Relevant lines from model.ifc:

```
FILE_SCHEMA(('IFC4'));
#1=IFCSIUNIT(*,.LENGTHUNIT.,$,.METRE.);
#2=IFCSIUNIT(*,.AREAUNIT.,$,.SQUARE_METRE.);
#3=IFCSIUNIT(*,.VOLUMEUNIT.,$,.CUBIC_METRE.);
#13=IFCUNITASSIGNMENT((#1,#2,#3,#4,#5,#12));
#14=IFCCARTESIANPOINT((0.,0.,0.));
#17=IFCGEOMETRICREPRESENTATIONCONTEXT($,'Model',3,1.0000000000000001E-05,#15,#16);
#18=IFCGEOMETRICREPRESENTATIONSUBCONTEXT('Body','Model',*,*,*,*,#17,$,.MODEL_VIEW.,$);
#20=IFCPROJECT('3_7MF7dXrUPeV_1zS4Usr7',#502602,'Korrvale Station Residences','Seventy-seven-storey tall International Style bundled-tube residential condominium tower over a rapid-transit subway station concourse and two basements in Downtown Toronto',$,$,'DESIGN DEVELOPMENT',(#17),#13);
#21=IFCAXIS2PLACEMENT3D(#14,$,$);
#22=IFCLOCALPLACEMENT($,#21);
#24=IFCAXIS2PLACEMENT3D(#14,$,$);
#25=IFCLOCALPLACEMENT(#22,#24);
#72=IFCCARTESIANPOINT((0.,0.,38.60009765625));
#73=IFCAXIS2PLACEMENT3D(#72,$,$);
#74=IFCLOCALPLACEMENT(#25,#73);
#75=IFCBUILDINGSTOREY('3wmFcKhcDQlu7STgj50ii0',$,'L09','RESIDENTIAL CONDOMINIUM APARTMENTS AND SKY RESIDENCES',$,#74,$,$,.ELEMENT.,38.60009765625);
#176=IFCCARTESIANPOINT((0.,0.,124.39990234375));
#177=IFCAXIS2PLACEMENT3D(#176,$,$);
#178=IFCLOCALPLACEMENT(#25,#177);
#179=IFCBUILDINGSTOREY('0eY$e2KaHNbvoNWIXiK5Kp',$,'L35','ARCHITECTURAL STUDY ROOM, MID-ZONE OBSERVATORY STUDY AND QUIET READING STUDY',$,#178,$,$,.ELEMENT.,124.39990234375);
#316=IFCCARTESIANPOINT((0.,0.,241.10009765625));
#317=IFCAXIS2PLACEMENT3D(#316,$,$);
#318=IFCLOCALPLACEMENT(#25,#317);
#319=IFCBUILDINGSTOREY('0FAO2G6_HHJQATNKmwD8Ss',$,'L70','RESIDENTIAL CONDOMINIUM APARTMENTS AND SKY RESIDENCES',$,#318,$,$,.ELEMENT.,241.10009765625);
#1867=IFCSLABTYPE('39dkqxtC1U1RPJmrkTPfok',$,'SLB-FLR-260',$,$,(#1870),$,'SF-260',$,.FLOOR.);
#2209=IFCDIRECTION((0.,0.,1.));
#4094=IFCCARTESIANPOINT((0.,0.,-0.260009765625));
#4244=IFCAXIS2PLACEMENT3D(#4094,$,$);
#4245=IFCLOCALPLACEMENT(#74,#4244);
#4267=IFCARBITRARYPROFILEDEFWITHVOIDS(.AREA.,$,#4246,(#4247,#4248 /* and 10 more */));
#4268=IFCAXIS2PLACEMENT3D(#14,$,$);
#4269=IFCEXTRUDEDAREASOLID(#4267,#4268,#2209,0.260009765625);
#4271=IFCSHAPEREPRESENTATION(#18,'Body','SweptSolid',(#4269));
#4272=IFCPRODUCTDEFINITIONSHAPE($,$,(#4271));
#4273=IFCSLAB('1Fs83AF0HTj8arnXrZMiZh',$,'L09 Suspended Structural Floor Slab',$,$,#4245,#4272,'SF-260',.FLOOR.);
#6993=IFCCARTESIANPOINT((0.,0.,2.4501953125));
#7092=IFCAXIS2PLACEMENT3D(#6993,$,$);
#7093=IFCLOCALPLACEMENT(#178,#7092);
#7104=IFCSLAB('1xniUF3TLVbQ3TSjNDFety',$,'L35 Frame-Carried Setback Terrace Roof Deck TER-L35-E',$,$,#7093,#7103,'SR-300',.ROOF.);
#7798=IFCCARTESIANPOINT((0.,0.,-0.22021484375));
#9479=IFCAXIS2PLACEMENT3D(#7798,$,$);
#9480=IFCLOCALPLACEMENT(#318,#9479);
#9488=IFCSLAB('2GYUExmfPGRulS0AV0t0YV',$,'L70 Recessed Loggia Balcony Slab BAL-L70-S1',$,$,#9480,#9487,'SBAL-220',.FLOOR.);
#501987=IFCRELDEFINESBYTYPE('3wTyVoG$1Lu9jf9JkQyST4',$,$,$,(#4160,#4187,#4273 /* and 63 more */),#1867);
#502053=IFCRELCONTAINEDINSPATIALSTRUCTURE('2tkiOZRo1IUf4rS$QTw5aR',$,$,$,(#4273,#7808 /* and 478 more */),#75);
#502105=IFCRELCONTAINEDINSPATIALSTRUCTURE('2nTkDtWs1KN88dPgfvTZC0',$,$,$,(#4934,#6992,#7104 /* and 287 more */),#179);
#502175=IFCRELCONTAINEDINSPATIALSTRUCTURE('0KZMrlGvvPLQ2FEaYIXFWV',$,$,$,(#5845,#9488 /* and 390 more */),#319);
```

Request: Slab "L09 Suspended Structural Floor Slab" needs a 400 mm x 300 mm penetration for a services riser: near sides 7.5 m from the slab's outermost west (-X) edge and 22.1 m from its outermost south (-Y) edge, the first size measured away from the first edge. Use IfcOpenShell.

```python
import numpy as np
import ifcopenshell
import ifcopenshell.api.feature
import ifcopenshell.api.geometry
import ifcopenshell.api.root
import ifcopenshell.geom
import ifcopenshell.util.placement
import ifcopenshell.util.representation
import ifcopenshell.util.shape
import ifcopenshell.util.unit

model = ifcopenshell.open("model.ifc")
unit_scale = ifcopenshell.util.unit.calculate_unit_scale(model)
settings = ifcopenshell.geom.settings()


def volume(element):
    """Net volume in cubic metres, openings subtracted."""
    shape = ifcopenshell.geom.create_shape(settings, element)
    return ifcopenshell.util.shape.get_volume(shape.geometry)


slab = model.by_id(4273)
before = volume(slab)

# Extent in the slab's own axes, in metres. The edges named are its -X and -Y sides.
slab_shape = ifcopenshell.geom.create_shape(settings, slab)
vertices = ifcopenshell.util.shape.get_vertices(slab_shape.geometry)
x_min, y_min, bottom = vertices.min(axis=0)
top = vertices[:, 2].max()

opening = ifcopenshell.api.root.create_entity(model, ifc_class="IfcOpeningElement", name="Services riser opening", predefined_type="OPENING")
context = ifcopenshell.util.representation.get_context(model, "Model", "Body", "MODEL_VIEW")
width, depth = 0.4, 0.3
outline = [(0.0, 0.0), (width, 0.0), (width, depth), (0.0, depth), (0.0, 0.0)]
# Overshoot both faces by 50 mm so the cut is clean.
shape = ifcopenshell.api.geometry.add_slab_representation(
    model, context=context, depth=top - bottom + 0.1, polyline=outline
)
ifcopenshell.api.geometry.assign_representation(model, product=opening, representation=shape)

matrix = ifcopenshell.util.placement.get_local_placement(slab.ObjectPlacement)
matrix[:, 3] = matrix @ np.append(np.array([x_min + 7.5, y_min + 22.1, bottom - 0.05]) / unit_scale, 1.0)
ifcopenshell.api.geometry.edit_object_placement(model, product=opening, matrix=matrix, is_si=False)
ifcopenshell.api.feature.add_feature(model, feature=opening, element=slab)

after = volume(slab)

print(f"slab volume {before:.3f} -> {after:.3f} m3")

model.write("model-out.ifc")
```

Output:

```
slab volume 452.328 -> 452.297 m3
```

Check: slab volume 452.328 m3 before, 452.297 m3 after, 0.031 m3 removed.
